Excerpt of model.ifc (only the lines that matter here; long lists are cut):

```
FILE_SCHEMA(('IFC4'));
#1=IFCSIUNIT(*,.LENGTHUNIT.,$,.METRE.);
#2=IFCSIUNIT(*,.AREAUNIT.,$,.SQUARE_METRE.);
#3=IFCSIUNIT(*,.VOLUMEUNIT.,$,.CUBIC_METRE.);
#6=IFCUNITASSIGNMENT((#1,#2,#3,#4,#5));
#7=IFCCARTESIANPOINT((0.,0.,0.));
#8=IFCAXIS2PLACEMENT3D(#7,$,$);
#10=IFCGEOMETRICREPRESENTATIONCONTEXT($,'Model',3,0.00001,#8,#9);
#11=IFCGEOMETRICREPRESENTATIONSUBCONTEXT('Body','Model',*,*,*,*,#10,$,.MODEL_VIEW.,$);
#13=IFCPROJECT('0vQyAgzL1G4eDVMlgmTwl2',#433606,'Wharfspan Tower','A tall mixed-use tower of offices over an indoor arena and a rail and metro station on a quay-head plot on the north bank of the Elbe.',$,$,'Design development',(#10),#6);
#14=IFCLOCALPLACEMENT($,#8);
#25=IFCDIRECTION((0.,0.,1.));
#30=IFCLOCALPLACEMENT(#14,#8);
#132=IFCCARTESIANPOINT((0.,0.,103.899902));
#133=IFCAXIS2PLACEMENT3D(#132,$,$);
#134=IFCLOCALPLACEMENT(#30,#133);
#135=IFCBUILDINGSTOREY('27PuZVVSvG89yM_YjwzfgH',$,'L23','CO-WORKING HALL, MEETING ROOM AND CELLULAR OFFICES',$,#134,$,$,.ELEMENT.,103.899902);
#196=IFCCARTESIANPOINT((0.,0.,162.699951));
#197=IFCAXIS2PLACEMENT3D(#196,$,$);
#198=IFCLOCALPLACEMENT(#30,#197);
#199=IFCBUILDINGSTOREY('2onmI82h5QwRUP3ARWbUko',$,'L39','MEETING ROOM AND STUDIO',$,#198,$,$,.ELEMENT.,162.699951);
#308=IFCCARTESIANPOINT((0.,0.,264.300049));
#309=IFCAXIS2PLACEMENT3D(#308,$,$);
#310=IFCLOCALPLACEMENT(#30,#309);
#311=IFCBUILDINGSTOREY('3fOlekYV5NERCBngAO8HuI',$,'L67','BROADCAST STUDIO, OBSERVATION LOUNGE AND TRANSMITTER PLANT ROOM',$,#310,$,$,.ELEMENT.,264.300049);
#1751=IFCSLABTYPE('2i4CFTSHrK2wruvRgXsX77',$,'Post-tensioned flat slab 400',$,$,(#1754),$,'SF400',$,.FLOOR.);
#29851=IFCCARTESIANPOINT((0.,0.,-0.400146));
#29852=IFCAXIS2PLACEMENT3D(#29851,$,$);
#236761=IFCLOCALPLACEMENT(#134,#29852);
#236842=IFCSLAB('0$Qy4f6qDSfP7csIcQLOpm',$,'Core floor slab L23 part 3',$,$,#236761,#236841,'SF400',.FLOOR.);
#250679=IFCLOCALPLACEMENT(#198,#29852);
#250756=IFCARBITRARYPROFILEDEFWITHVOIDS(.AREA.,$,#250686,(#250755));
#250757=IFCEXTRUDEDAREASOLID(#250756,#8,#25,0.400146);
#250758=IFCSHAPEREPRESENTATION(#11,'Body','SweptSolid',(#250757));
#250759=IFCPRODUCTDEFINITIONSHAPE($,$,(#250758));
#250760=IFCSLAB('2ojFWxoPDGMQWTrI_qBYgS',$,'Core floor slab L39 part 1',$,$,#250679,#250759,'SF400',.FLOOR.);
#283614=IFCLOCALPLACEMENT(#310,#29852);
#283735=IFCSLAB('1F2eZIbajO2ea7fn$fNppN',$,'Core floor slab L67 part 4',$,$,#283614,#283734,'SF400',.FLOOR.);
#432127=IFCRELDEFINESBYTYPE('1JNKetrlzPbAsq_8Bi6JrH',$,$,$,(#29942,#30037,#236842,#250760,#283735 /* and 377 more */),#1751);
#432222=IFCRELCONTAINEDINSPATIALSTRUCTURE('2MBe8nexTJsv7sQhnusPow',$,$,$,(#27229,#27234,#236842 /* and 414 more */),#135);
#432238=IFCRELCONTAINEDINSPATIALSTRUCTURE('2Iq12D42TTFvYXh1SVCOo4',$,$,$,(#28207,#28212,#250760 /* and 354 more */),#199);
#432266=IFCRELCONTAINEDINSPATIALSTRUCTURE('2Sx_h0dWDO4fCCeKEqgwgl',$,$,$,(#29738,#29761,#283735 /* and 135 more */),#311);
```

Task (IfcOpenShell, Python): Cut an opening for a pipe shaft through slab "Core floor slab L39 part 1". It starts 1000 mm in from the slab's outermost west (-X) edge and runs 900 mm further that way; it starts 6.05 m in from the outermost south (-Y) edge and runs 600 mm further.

```python
import numpy as np
import ifcopenshell
import ifcopenshell.api.feature
import ifcopenshell.api.geometry
import ifcopenshell.api.root
import ifcopenshell.geom
import ifcopenshell.util.placement
import ifcopenshell.util.representation
import ifcopenshell.util.shape
import ifcopenshell.util.unit

model = ifcopenshell.open("model.ifc")
unit_scale = ifcopenshell.util.unit.calculate_unit_scale(model)
settings = ifcopenshell.geom.settings()


def volume(element):
    """Net volume in cubic metres, openings subtracted."""
    shape = ifcopenshell.geom.create_shape(settings, element)
    return ifcopenshell.util.shape.get_volume(shape.geometry)


slab = model.by_guid("2ojFWxoPDGMQWTrI_qBYgS")
before = volume(slab)

# Extent in the slab's own axes, in metres. The edges named are its -X and -Y sides.
slab_shape = ifcopenshell.geom.create_shape(settings, slab)
vertices = ifcopenshell.util.shape.get_vertices(slab_shape.geometry)
x_min, y_min, bottom = vertices.min(axis=0)
top = vertices[:, 2].max()

opening = ifcopenshell.api.root.create_entity(model, ifc_class="IfcOpeningElement", name="Pipe shaft opening", predefined_type="OPENING")
context = ifcopenshell.util.representation.get_context(model, "Model", "Body", "MODEL_VIEW")
width, depth = 0.9, 0.6
outline = [(0.0, 0.0), (width, 0.0), (width, depth), (0.0, depth), (0.0, 0.0)]
# Overshoot both faces by 50 mm so the cut is clean.
shape = ifcopenshell.api.geometry.add_slab_representation(
    model, context=context, depth=top - bottom + 0.1, polyline=outline
)
ifcopenshell.api.geometry.assign_representation(model, product=opening, representation=shape)

matrix = ifcopenshell.util.placement.get_local_placement(slab.ObjectPlacement)
matrix[:, 3] = matrix @ np.append(np.array([x_min + 1, y_min + 6.05, bottom - 0.05]) / unit_scale, 1.0)
ifcopenshell.api.geometry.edit_object_placement(model, product=opening, matrix=matrix, is_si=False)
ifcopenshell.api.feature.add_feature(model, feature=opening, element=slab)

after = volume(slab)

print(f"slab volume {before:.3f} -> {after:.3f} m3")

model.write("model-out.ifc")
```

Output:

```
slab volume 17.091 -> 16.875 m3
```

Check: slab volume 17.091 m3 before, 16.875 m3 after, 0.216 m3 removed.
